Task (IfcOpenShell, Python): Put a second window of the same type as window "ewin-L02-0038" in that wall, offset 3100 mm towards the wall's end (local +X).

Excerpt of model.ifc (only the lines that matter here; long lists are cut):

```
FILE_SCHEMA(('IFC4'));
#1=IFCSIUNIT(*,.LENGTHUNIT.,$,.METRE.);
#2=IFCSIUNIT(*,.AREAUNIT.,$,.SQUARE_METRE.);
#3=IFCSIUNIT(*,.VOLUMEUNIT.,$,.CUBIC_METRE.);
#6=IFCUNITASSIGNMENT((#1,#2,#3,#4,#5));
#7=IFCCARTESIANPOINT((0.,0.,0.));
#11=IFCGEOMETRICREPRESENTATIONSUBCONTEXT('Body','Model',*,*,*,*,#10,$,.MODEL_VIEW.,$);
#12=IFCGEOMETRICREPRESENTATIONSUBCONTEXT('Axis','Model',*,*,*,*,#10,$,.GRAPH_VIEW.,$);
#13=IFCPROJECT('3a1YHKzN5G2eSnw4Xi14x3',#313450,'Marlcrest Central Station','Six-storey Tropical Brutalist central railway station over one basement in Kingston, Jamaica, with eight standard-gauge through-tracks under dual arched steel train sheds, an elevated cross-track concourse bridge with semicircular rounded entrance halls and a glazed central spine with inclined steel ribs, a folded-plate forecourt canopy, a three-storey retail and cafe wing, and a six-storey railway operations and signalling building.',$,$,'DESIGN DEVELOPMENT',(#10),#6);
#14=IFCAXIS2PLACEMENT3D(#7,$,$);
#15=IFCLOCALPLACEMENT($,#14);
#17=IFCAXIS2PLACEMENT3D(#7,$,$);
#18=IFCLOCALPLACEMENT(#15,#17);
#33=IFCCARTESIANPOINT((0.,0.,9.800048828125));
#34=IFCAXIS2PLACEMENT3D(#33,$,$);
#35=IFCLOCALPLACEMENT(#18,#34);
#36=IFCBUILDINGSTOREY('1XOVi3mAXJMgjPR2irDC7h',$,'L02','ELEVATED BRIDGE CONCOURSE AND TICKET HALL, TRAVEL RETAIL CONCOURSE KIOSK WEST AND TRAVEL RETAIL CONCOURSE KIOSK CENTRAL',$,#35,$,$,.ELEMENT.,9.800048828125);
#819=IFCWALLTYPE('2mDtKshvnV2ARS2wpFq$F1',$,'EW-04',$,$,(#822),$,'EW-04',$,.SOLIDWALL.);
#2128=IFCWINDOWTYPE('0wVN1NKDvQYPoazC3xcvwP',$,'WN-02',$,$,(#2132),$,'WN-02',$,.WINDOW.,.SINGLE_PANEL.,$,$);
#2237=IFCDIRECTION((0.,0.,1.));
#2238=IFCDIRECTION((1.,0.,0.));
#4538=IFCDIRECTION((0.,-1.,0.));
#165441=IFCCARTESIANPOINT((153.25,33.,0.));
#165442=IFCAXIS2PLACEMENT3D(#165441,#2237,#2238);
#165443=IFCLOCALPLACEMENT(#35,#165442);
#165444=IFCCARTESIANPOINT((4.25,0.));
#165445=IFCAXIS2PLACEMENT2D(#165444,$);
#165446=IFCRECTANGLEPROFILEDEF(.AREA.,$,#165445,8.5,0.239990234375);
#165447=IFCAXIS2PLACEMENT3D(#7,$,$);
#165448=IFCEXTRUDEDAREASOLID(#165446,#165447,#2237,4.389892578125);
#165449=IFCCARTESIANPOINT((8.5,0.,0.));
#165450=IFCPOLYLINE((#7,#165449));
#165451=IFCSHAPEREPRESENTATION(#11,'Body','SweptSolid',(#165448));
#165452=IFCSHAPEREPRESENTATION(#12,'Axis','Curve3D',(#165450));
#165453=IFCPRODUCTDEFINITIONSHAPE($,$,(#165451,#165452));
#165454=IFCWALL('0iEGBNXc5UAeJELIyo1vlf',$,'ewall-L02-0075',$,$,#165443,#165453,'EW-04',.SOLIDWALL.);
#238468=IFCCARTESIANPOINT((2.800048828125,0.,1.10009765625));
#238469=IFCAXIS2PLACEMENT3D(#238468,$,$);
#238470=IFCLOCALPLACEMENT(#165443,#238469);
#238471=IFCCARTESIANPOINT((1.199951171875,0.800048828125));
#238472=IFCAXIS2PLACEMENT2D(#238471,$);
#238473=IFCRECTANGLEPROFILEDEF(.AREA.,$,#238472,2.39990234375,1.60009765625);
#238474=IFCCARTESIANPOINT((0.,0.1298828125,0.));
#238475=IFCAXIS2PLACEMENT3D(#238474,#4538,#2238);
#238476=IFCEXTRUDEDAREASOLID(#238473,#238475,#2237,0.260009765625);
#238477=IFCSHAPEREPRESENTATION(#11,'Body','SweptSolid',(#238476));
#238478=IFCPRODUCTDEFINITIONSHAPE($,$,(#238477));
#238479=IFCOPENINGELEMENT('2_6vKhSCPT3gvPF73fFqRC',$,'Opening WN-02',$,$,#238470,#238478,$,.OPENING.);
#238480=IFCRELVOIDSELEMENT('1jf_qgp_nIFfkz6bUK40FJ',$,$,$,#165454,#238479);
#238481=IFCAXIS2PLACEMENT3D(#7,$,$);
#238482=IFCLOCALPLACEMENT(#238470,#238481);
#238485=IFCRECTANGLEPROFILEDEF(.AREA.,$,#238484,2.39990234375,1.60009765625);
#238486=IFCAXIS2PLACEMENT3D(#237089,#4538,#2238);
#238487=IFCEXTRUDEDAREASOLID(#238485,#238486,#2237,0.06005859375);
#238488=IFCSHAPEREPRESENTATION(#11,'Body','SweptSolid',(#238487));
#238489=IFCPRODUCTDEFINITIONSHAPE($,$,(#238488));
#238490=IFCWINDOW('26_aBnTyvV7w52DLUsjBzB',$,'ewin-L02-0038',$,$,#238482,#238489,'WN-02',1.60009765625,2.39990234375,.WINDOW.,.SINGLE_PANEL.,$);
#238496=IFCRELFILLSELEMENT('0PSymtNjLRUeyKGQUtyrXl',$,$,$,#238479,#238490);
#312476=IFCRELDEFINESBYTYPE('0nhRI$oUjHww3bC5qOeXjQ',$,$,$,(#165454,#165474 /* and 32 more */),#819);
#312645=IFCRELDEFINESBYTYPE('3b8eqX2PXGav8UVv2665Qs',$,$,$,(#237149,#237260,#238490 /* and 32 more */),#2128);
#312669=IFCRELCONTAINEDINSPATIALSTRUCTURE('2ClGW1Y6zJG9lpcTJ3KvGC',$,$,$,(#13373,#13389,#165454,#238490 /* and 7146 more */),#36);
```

```python
import ifcopenshell
import ifcopenshell.api.feature
import ifcopenshell.api.geometry
import ifcopenshell.api.root
import ifcopenshell.geom
import ifcopenshell.util.element
import ifcopenshell.util.placement
import ifcopenshell.util.shape
import ifcopenshell.util.unit

model = ifcopenshell.open("model.ifc")
unit_scale = ifcopenshell.util.unit.calculate_unit_scale(model)
settings = ifcopenshell.geom.settings()


def volume(element):
    """Net volume in cubic metres, openings subtracted."""
    shape = ifcopenshell.geom.create_shape(settings, element)
    return ifcopenshell.util.shape.get_volume(shape.geometry)


window = model.by_id(238490)
opening = window.FillsVoids[0].RelatingOpeningElement
wall = opening.VoidsElements[0].RelatingBuildingElement
before = volume(wall)
shift = ifcopenshell.util.placement.get_local_placement(wall.ObjectPlacement)[:3, 0] * 3.1 / unit_scale

# copy_class copies the void relationship, type, container and properties, but no geometry.
new_opening = ifcopenshell.api.root.copy_class(model, product=opening)
new_opening.Representation = ifcopenshell.util.element.copy_deep(
    model, opening.Representation, exclude=["IfcGeometricRepresentationContext", "IfcRepresentationMap"]
)
new_window = ifcopenshell.api.root.copy_class(model, product=window)
new_window.Representation = ifcopenshell.util.element.copy_deep(
    model, window.Representation, exclude=["IfcGeometricRepresentationContext", "IfcRepresentationMap"]
)
new_window.Tag = None
ifcopenshell.api.feature.add_filling(model, opening=new_opening, element=new_window)

for old, new in ((opening, new_opening), (window, new_window)):
    matrix = ifcopenshell.util.placement.get_local_placement(old.ObjectPlacement)
    matrix[:3, 3] += shift
    ifcopenshell.api.geometry.edit_object_placement(model, product=new, matrix=matrix, is_si=False)

after = volume(wall)

print(f"wall volume {before:.3f} -> {after:.3f} m3")

model.write("model_updated.ifc")
```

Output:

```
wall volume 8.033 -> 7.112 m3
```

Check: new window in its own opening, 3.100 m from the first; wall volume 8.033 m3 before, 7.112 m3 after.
